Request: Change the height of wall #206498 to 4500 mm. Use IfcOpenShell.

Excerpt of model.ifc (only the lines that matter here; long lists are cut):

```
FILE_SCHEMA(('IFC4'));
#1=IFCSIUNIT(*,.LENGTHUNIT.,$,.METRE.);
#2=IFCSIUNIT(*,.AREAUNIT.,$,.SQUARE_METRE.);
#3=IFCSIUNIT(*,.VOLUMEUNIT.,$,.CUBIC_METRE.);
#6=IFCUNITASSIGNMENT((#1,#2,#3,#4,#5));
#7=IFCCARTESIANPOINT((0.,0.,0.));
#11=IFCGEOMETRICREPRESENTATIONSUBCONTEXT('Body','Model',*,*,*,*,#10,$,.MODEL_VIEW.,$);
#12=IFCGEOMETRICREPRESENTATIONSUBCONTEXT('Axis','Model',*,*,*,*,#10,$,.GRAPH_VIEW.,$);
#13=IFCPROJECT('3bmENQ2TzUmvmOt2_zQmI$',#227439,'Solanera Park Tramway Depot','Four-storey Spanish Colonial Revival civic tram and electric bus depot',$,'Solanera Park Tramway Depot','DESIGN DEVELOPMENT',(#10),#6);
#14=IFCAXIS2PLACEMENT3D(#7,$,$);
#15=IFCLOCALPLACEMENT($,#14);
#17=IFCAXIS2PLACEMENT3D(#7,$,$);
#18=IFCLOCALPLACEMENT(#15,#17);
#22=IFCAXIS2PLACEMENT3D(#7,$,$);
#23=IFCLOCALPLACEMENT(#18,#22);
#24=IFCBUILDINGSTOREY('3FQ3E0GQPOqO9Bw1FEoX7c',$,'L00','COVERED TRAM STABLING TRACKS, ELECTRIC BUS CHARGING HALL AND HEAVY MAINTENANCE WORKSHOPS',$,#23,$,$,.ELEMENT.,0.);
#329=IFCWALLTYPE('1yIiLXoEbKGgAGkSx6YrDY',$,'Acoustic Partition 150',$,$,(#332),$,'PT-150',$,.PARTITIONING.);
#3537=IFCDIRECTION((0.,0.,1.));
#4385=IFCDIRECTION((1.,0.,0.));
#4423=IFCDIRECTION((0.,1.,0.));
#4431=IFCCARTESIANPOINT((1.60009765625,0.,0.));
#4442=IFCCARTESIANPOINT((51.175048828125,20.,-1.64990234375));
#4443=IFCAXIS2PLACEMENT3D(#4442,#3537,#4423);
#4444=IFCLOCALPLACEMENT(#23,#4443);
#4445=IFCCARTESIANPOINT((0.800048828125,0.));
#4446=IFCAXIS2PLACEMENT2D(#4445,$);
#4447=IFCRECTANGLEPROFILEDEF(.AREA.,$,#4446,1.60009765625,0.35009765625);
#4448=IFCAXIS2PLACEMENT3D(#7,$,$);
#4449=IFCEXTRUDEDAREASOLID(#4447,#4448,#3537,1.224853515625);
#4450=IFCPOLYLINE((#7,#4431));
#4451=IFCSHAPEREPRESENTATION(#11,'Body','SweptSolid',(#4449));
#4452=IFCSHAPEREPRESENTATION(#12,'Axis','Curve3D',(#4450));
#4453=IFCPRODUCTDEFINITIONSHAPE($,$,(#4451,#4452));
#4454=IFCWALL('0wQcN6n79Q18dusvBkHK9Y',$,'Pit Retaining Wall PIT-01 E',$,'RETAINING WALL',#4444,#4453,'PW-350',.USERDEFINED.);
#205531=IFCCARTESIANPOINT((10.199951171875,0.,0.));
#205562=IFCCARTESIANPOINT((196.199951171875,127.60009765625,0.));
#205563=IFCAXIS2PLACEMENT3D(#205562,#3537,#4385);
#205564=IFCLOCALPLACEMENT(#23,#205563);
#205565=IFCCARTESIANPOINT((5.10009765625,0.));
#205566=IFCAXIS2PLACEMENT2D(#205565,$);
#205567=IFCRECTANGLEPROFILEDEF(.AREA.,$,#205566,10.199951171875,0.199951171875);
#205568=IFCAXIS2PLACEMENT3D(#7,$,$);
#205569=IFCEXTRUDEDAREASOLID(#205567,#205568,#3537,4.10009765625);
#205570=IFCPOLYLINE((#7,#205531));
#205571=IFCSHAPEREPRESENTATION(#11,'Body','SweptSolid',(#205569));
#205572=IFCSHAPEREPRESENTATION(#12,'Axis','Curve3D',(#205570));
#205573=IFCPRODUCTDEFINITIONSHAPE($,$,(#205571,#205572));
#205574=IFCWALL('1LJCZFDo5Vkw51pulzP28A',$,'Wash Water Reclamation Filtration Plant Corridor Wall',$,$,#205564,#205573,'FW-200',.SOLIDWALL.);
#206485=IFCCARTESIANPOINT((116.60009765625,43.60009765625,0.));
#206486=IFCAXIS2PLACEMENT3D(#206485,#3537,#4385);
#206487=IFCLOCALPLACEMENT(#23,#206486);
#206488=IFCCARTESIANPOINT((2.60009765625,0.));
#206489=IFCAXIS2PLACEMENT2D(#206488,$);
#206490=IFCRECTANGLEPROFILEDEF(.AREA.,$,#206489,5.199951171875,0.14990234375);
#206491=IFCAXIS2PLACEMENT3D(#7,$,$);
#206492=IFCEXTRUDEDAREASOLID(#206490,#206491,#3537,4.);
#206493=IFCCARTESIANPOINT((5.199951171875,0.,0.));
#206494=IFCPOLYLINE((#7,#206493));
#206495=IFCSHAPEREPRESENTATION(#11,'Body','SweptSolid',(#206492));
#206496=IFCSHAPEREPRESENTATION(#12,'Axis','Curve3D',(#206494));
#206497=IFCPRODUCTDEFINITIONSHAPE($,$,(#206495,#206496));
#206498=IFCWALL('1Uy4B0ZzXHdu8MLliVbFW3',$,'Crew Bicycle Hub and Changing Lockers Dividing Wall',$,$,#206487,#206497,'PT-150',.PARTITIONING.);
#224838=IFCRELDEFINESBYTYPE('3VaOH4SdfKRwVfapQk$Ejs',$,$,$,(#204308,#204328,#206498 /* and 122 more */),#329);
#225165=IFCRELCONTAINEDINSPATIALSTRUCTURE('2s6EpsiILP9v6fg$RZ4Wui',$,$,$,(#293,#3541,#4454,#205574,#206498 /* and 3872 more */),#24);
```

```python
import ifcopenshell
import ifcopenshell.geom
import ifcopenshell.util.representation
import ifcopenshell.util.shape
import ifcopenshell.util.unit

model = ifcopenshell.open("model.ifc")
unit_scale = ifcopenshell.util.unit.calculate_unit_scale(model)
settings = ifcopenshell.geom.settings()


def volume(element):
    """Net volume in cubic metres, openings subtracted."""
    shape = ifcopenshell.geom.create_shape(settings, element)
    return ifcopenshell.util.shape.get_volume(shape.geometry)


wall = model.by_id(206498)
before = volume(wall)

body = ifcopenshell.util.representation.get_representation(wall, "Model", "Body")
solid = body.Items[0]
old_height = solid.Depth
solid.Depth = 4.5 / unit_scale
after = volume(wall)

print(f"height {old_height:g} -> {solid.Depth:g}, volume {before:.3f} -> {after:.3f} m3")

model.write("model_edited.ifc")
```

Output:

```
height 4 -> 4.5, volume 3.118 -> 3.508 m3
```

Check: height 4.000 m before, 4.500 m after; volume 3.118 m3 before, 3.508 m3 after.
